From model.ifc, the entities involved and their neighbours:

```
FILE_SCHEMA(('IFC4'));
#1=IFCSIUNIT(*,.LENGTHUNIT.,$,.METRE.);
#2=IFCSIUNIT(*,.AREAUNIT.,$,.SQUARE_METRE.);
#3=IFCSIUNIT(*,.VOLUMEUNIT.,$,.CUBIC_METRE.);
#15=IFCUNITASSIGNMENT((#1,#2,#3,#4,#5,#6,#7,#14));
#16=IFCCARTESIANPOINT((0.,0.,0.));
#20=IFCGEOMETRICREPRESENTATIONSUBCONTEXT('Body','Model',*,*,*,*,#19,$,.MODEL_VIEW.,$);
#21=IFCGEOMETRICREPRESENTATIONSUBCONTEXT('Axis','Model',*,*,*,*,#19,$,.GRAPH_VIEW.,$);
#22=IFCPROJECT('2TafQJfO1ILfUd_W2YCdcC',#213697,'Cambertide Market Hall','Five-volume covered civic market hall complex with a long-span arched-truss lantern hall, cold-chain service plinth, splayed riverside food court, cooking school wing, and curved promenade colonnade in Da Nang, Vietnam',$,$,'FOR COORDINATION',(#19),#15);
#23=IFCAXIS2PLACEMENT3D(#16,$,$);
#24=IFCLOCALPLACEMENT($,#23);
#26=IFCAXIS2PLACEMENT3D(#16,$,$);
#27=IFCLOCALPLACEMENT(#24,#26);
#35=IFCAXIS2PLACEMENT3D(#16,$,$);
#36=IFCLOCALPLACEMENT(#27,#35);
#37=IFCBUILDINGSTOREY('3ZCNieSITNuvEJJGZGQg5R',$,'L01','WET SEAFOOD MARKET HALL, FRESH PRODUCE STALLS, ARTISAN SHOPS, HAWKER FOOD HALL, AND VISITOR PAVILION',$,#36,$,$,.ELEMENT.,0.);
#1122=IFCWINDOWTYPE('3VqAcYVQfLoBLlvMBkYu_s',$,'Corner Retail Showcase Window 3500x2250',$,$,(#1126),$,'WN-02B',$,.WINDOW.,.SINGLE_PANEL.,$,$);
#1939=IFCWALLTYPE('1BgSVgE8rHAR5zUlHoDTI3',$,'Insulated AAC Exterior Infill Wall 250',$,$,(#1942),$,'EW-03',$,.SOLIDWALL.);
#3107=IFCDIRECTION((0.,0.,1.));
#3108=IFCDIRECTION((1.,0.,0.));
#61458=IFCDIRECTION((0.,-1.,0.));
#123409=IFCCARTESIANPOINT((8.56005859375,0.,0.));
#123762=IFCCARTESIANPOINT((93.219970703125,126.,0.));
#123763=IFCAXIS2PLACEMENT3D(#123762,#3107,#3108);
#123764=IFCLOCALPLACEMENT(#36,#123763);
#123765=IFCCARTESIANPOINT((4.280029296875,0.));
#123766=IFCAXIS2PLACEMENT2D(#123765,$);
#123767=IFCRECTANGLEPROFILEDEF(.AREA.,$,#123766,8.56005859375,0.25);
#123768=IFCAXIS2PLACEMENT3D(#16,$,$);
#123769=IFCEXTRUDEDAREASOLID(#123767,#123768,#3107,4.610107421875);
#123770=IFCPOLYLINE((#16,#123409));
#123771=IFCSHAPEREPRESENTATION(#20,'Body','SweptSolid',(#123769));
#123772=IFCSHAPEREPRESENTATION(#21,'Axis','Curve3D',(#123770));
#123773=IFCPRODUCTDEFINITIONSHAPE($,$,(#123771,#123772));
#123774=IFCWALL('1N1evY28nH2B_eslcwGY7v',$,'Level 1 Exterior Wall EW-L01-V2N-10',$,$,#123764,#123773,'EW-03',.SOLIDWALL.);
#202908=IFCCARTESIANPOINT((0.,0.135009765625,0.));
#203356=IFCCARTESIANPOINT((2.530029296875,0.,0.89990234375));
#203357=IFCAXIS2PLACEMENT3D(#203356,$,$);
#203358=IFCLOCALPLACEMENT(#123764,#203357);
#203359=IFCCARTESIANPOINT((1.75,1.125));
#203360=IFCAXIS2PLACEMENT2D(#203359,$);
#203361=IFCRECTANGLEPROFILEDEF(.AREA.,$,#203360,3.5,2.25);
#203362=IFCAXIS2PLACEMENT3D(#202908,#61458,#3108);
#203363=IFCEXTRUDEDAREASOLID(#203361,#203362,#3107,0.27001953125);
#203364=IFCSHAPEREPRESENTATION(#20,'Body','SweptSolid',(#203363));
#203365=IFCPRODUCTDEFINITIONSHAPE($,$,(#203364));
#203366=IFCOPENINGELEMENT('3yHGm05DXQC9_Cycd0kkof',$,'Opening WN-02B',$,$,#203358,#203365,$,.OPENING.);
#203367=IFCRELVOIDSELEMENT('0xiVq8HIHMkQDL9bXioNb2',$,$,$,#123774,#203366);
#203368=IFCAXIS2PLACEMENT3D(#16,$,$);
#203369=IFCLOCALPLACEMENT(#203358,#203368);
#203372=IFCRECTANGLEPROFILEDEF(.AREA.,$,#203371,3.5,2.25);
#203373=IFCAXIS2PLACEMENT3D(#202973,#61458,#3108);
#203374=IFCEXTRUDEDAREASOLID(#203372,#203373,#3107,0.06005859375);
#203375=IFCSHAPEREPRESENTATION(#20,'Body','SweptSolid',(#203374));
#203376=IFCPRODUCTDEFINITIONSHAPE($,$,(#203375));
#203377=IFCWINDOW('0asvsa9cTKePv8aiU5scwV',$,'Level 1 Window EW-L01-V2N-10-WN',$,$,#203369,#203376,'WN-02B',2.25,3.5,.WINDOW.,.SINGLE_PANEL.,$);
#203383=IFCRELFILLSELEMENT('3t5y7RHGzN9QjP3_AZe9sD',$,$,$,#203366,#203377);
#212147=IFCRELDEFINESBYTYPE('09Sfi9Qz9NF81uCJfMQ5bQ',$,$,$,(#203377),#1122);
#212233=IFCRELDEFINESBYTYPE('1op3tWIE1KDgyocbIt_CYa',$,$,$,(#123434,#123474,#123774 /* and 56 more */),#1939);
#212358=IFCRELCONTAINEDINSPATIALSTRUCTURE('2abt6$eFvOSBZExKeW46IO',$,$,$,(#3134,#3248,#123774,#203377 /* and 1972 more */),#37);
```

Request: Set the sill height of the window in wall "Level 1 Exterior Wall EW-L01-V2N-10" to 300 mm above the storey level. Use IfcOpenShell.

```python
import numpy as np
import ifcopenshell
import ifcopenshell.api.geometry
import ifcopenshell.geom
import ifcopenshell.util.element
import ifcopenshell.util.placement
import ifcopenshell.util.shape
import ifcopenshell.util.unit

model = ifcopenshell.open("model.ifc")
unit_scale = ifcopenshell.util.unit.calculate_unit_scale(model)

window = model.by_guid("0asvsa9cTKePv8aiU5scwV")
opening = window.FillsVoids[0].RelatingOpeningElement
storey = ifcopenshell.util.element.get_container(window, ifc_class="IfcBuildingStorey")
level = ifcopenshell.util.placement.get_local_placement(storey.ObjectPlacement)[2, 3]

# The opening's origin need not be at the sill, so measure its lowest point.
shape = ifcopenshell.geom.create_shape(ifcopenshell.geom.settings(), opening)
bottom = ifcopenshell.util.shape.get_shape_bottom_elevation(shape, shape.geometry) / unit_scale
dz = level + 0.3 - bottom

shift = np.array([0.0, 0.0, dz])
# The window is placed relative to its opening, so it follows when the opening moves.
matrix = ifcopenshell.util.placement.get_local_placement(opening.ObjectPlacement)
matrix[:3, 3] += shift
ifcopenshell.api.geometry.edit_object_placement(
    model, product=opening, matrix=matrix, is_si=False, should_transform_children=True
)

print(f"moved by {dz * unit_scale:+.3f} m")

model.write("model_rev.ifc")
```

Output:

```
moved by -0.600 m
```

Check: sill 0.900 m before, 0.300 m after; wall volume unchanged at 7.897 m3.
